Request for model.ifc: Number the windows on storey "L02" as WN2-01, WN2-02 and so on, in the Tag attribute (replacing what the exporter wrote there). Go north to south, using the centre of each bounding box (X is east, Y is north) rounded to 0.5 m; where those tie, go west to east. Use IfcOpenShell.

First a look at what the model holds.

```python
import ifcopenshell
import ifcopenshell.util.element
import ifcopenshell.util.placement

model = ifcopenshell.open("model.ifc")
print(model.schema)
storey = next(s for s in model.by_type("IfcBuildingStorey") if s.Name == "L02")
windows = [e for e in ifcopenshell.util.element.get_decomposition(storey) if e.is_a("IfcWindow")]
for e in sorted(windows, key=lambda e: e.id()):
    origin = ifcopenshell.util.placement.get_local_placement(e.ObjectPlacement)[:3, 3]
    print(e.id(), e.Tag, e.Name, origin.round(2) + 0.0, sep=" | ")
```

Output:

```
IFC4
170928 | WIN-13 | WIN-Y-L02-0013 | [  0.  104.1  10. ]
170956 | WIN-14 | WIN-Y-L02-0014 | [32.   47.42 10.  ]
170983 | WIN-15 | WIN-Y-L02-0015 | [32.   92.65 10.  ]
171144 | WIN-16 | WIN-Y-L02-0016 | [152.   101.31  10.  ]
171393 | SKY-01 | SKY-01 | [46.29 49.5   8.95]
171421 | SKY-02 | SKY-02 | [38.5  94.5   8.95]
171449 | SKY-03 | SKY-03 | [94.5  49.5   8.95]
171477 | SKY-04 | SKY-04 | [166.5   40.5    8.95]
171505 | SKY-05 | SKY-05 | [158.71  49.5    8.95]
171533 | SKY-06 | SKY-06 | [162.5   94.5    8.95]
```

```python
import ifcopenshell
import ifcopenshell.geom
import ifcopenshell.util.element
import ifcopenshell.util.shape

model = ifcopenshell.open("model.ifc")
settings = ifcopenshell.geom.settings()
settings.set("use-world-coords", True)


def centre(element):
    shape = ifcopenshell.geom.create_shape(settings, element)
    return ifcopenshell.util.shape.get_bbox_centroid(shape.geometry)


storey = next(s for s in model.by_type("IfcBuildingStorey") if s.Name == "L02")
windows = [e for e in ifcopenshell.util.element.get_decomposition(storey) if e.is_a("IfcWindow")]

# Insertion points can sit at a corner or the storey origin, so sort by the geometry (in metres).
centres = {e: centre(e) for e in windows}
windows.sort(key=lambda e: (-round(centres[e][1] / 0.5), centres[e][0]))

for i, e in enumerate(windows, start=1):
    number = f"WN2-{i:02d}"
    e.Tag = number
    print(e.id(), number)

model.write("model_edited.ifc")
```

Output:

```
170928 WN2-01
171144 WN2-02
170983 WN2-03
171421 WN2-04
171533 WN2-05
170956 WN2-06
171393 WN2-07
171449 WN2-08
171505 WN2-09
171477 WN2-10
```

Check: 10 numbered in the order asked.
